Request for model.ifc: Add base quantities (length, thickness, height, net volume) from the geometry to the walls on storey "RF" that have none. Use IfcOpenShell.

First a look at what the model holds.

```python
import ifcopenshell
import ifcopenshell.util.element
import ifcopenshell.util.unit

model = ifcopenshell.open("model.ifc")
print(model.schema)
for unit_type in ("LENGTHUNIT", "AREAUNIT", "VOLUMEUNIT"):
    print(unit_type, ifcopenshell.util.unit.calculate_unit_scale(model, unit_type))
storey = next(s for s in model.by_type("IfcBuildingStorey") if s.Name == "RF")
walls = [e for e in ifcopenshell.util.element.get_decomposition(storey) if e.is_a("IfcWall")]
for e in sorted(walls, key=lambda e: e.id()):
    print(e.id(), e.is_a(), e.Name, list(ifcopenshell.util.element.get_psets(e, qtos_only=True)), sep=" | ")
```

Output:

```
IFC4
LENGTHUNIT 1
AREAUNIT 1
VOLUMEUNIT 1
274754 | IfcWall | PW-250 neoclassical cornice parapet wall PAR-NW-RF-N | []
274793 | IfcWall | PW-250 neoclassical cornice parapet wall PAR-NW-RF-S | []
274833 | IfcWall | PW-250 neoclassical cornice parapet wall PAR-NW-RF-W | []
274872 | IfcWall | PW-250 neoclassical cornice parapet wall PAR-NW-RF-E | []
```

```python
import ifcopenshell
import ifcopenshell.api.pset
import ifcopenshell.geom
import ifcopenshell.util.element
import ifcopenshell.util.shape
import ifcopenshell.util.unit

model = ifcopenshell.open("model.ifc")
unit_scale = ifcopenshell.util.unit.calculate_unit_scale(model)
volume_scale = ifcopenshell.util.unit.calculate_unit_scale(model, "VOLUMEUNIT")
settings = ifcopenshell.geom.settings()

storey = next(s for s in model.by_type("IfcBuildingStorey") if s.Name == "RF")
walls = [e for e in ifcopenshell.util.element.get_decomposition(storey) if e.is_a("IfcWall")]

for e in sorted(walls, key=lambda e: e.id()):
    if ifcopenshell.util.element.get_psets(e, qtos_only=True, should_inherit=False):
        continue
    # Geometry comes back in metres, in the element's own axes.
    shape = ifcopenshell.geom.create_shape(settings, e)
    values = {
        "Length": ifcopenshell.util.shape.get_x(shape.geometry) / unit_scale,
        "Width": ifcopenshell.util.shape.get_y(shape.geometry) / unit_scale,
        "Height": ifcopenshell.util.shape.get_z(shape.geometry) / unit_scale,
        "NetVolume": ifcopenshell.util.shape.get_volume(shape.geometry) / volume_scale,
    }
    qto = ifcopenshell.api.pset.add_qto(model, product=e, name="Qto_WallBaseQuantities")
    ifcopenshell.api.pset.edit_qto(model, qto=qto, properties=values)
    print(e.id(), {k: round(v, 3) for k, v in values.items()})

model.write("model_updated.ifc")
```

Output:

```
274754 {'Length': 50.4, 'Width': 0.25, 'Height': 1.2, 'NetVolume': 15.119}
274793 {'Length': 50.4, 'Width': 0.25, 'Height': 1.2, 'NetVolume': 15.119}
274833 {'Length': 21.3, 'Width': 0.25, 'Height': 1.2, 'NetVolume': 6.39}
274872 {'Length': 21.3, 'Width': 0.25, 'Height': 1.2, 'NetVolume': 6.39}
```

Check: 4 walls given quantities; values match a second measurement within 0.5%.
